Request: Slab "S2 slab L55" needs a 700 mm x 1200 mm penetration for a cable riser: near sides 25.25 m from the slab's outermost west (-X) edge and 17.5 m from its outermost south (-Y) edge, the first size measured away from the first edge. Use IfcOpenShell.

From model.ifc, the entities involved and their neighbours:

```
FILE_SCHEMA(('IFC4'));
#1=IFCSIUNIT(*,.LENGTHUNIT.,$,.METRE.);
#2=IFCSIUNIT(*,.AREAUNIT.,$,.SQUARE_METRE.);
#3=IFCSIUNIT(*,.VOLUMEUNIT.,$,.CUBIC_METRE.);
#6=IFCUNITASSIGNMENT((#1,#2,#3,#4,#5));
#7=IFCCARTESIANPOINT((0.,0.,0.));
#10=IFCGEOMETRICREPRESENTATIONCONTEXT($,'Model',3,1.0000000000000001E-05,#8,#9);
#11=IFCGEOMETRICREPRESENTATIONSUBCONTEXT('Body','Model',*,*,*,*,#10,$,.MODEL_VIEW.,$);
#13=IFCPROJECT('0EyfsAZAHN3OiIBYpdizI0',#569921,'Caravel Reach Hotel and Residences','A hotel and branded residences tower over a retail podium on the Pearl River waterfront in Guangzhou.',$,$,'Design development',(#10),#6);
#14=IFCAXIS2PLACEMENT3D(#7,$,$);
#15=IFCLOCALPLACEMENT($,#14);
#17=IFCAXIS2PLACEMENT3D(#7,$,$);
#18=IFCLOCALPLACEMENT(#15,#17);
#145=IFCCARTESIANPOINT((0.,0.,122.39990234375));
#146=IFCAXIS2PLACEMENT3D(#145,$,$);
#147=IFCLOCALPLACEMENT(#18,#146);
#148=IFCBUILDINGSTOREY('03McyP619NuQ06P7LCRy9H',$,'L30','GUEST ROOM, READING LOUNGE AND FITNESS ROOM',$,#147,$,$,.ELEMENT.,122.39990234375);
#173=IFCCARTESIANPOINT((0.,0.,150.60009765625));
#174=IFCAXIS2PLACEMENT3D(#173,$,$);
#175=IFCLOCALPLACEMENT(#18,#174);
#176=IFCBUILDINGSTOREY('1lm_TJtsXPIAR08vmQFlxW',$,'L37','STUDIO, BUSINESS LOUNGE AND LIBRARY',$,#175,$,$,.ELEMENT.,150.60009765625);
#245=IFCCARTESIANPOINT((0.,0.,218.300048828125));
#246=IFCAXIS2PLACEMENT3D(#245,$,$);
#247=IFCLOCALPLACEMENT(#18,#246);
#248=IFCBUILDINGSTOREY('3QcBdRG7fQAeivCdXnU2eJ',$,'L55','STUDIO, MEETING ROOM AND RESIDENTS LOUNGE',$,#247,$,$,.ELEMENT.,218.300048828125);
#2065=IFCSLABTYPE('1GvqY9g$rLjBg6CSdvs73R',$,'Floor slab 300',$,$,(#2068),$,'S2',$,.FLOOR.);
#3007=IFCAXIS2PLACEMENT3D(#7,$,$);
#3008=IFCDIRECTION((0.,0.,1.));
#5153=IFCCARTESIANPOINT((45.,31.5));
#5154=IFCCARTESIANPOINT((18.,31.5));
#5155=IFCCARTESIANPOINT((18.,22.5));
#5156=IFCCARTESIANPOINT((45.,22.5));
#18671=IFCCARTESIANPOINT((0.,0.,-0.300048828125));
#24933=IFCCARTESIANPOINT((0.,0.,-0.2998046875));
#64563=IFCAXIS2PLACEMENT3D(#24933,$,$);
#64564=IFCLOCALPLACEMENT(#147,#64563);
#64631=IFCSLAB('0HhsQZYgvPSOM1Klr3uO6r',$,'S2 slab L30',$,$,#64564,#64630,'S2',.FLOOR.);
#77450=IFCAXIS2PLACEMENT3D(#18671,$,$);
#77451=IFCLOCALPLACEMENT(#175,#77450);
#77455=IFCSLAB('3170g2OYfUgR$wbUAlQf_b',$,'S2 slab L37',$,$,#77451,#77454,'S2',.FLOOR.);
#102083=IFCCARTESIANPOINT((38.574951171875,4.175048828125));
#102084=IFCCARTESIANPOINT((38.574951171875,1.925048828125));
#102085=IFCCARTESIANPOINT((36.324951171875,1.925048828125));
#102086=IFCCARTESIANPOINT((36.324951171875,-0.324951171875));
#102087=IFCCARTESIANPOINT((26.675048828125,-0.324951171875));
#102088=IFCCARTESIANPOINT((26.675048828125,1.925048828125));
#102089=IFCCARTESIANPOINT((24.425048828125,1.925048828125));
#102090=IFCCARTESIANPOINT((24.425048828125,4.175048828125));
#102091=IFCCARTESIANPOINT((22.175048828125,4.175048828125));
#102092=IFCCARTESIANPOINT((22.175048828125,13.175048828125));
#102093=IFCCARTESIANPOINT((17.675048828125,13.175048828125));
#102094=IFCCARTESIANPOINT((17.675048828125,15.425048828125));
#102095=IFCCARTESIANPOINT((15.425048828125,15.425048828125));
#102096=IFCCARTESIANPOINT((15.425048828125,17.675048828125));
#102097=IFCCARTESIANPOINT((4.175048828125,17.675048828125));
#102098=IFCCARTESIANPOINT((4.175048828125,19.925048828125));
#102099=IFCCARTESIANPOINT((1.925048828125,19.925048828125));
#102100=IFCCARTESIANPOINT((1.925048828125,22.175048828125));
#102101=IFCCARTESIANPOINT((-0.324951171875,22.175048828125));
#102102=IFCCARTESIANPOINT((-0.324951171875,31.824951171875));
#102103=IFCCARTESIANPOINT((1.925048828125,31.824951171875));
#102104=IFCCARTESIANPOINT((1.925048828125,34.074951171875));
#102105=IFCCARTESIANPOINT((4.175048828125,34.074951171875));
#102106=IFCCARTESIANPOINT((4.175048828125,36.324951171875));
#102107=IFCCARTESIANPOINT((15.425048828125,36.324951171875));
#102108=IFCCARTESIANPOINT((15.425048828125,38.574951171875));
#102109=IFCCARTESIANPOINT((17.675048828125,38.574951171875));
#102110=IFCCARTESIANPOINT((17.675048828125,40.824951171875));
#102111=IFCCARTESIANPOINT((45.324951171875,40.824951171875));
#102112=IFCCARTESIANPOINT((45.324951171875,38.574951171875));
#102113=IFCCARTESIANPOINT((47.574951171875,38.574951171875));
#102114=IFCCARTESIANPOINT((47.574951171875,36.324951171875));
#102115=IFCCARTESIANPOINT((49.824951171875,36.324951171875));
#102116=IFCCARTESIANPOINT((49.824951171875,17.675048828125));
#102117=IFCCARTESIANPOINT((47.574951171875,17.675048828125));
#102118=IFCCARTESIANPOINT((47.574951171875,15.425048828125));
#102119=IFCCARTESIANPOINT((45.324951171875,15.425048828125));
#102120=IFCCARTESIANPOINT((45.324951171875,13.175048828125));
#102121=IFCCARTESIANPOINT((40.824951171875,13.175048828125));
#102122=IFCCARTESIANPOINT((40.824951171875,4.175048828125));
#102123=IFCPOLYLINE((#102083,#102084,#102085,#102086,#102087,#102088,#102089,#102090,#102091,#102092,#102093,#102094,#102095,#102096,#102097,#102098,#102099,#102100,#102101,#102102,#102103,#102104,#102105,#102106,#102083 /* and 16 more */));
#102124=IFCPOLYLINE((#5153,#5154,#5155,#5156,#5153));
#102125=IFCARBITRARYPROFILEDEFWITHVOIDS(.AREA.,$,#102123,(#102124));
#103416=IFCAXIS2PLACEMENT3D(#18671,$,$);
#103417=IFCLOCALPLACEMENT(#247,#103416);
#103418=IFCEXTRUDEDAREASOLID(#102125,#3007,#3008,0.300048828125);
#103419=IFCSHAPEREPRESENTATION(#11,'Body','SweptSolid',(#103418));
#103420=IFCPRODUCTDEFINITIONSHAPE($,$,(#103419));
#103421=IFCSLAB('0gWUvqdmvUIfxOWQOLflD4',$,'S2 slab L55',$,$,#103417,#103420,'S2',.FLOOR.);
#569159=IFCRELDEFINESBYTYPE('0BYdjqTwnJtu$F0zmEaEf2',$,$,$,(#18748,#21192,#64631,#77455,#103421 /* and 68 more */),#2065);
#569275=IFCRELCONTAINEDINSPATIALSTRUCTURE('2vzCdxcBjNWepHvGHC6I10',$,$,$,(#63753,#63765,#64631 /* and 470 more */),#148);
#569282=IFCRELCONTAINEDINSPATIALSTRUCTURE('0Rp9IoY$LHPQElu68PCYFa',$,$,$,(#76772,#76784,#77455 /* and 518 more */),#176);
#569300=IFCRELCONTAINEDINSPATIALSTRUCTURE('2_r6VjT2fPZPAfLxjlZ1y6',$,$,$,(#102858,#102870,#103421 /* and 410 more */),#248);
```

```python
import numpy as np
import ifcopenshell
import ifcopenshell.api.feature
import ifcopenshell.api.geometry
import ifcopenshell.api.root
import ifcopenshell.geom
import ifcopenshell.util.placement
import ifcopenshell.util.representation
import ifcopenshell.util.shape
import ifcopenshell.util.unit

model = ifcopenshell.open("model.ifc")
unit_scale = ifcopenshell.util.unit.calculate_unit_scale(model)
settings = ifcopenshell.geom.settings()


def volume(element):
    """Net volume in cubic metres, openings subtracted."""
    shape = ifcopenshell.geom.create_shape(settings, element)
    return ifcopenshell.util.shape.get_volume(shape.geometry)


slab = model.by_guid("0gWUvqdmvUIfxOWQOLflD4")
before = volume(slab)

# Extent in the slab's own axes, in metres. The edges named are its -X and -Y sides.
slab_shape = ifcopenshell.geom.create_shape(settings, slab)
vertices = ifcopenshell.util.shape.get_vertices(slab_shape.geometry)
x_min, y_min, bottom = vertices.min(axis=0)
top = vertices[:, 2].max()

opening = ifcopenshell.api.root.create_entity(model, ifc_class="IfcOpeningElement", name="Cable riser opening", predefined_type="OPENING")
context = ifcopenshell.util.representation.get_context(model, "Model", "Body", "MODEL_VIEW")
width, depth = 0.7, 1.2
outline = [(0.0, 0.0), (width, 0.0), (width, depth), (0.0, depth), (0.0, 0.0)]
# Overshoot both faces by 50 mm so the cut is clean.
shape = ifcopenshell.api.geometry.add_slab_representation(
    model, context=context, depth=top - bottom + 0.1, polyline=outline
)
ifcopenshell.api.geometry.assign_representation(model, product=opening, representation=shape)

matrix = ifcopenshell.util.placement.get_local_placement(slab.ObjectPlacement)
matrix[:, 3] = matrix @ np.append(np.array([x_min + 25.25, y_min + 17.5, bottom - 0.05]) / unit_scale, 1.0)
ifcopenshell.api.geometry.edit_object_placement(model, product=opening, matrix=matrix, is_si=False)
ifcopenshell.api.feature.add_feature(model, feature=opening, element=slab)

after = volume(slab)

print(f"slab volume {before:.3f} -> {after:.3f} m3")

model.write("model_v2.ifc")
```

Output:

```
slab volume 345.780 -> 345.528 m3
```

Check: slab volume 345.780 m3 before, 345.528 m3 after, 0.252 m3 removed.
